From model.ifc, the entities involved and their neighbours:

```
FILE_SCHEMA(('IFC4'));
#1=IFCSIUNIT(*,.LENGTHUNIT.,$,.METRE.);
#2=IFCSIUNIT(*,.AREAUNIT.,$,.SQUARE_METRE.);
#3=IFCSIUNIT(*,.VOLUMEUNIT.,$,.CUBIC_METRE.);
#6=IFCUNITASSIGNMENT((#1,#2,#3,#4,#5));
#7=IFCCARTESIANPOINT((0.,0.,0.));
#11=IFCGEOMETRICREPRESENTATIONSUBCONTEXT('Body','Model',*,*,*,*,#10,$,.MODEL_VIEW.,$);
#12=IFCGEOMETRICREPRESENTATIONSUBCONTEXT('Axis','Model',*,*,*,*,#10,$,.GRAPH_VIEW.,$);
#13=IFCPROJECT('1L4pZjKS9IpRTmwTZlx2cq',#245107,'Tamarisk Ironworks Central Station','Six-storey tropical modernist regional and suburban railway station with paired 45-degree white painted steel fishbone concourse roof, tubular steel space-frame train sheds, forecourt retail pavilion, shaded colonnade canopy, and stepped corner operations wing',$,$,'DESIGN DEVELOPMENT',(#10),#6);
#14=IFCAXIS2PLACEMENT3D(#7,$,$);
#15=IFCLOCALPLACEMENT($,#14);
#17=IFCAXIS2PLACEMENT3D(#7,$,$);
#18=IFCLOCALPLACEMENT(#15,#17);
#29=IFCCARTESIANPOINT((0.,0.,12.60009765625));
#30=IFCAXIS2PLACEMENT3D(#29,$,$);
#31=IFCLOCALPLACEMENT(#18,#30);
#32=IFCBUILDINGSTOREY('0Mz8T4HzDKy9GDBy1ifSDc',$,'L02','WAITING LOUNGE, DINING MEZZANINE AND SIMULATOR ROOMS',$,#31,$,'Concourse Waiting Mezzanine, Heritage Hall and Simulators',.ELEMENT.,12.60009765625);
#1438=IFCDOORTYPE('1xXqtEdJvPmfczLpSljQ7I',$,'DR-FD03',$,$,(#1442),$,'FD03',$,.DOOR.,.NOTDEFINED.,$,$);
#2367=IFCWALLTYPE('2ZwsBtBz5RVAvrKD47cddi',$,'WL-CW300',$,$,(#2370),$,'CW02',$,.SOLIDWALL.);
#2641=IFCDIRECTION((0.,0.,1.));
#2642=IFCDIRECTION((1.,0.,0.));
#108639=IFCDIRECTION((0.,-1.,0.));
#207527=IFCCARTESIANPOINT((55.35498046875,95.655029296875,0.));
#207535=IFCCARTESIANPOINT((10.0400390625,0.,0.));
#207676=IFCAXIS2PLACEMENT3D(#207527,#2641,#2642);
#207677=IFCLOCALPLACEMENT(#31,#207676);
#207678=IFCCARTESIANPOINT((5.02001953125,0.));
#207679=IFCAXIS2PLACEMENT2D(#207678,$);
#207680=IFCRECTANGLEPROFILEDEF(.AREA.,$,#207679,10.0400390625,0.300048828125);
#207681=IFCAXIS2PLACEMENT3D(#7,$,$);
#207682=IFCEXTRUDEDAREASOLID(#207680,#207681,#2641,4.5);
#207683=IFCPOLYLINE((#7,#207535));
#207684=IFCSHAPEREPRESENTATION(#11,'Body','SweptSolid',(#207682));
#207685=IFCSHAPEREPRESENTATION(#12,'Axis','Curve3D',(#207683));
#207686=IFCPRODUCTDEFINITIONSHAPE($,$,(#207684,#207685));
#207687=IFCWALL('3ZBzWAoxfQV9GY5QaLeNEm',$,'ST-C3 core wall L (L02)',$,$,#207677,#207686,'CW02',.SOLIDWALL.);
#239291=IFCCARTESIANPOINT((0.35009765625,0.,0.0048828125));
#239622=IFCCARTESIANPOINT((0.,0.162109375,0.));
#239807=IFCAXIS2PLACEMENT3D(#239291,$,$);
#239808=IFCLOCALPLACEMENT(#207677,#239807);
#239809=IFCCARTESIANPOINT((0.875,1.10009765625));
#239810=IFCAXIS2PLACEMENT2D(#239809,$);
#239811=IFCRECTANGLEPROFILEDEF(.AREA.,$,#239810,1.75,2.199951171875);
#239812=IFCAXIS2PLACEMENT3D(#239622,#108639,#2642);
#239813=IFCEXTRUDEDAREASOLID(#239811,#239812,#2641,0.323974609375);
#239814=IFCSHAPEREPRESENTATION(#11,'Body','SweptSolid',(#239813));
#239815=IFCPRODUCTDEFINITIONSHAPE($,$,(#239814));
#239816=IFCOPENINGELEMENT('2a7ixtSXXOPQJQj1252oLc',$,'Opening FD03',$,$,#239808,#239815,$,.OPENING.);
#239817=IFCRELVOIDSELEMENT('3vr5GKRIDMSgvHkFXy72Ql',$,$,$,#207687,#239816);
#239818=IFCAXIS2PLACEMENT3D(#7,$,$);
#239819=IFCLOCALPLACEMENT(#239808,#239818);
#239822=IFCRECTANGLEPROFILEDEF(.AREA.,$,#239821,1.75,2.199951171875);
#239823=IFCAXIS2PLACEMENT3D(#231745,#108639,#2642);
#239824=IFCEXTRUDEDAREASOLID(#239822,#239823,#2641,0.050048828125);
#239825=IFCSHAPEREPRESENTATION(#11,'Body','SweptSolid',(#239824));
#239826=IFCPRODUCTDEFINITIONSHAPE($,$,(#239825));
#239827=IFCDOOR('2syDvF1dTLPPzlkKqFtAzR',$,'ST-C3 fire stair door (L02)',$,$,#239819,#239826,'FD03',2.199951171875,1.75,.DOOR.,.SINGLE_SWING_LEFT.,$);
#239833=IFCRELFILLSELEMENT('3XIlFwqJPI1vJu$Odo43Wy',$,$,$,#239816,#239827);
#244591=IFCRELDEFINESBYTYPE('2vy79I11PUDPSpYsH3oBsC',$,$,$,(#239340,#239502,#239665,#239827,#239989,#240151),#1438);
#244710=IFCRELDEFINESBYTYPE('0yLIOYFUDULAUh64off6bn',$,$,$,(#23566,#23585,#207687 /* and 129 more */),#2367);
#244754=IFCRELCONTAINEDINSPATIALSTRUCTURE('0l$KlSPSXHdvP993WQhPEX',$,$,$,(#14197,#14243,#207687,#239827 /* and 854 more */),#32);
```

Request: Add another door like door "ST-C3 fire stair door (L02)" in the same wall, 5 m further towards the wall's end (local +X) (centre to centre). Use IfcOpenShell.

```python
import ifcopenshell
import ifcopenshell.api.feature
import ifcopenshell.api.geometry
import ifcopenshell.api.root
import ifcopenshell.geom
import ifcopenshell.util.element
import ifcopenshell.util.placement
import ifcopenshell.util.shape
import ifcopenshell.util.unit

model = ifcopenshell.open("model.ifc")
unit_scale = ifcopenshell.util.unit.calculate_unit_scale(model)
settings = ifcopenshell.geom.settings()


def volume(element):
    """Net volume in cubic metres, openings subtracted."""
    shape = ifcopenshell.geom.create_shape(settings, element)
    return ifcopenshell.util.shape.get_volume(shape.geometry)


door = model.by_guid("2syDvF1dTLPPzlkKqFtAzR")
opening = door.FillsVoids[0].RelatingOpeningElement
wall = opening.VoidsElements[0].RelatingBuildingElement
before = volume(wall)
shift = ifcopenshell.util.placement.get_local_placement(wall.ObjectPlacement)[:3, 0] * 5 / unit_scale

# copy_class copies the void relationship, type, container and properties, but no geometry.
new_opening = ifcopenshell.api.root.copy_class(model, product=opening)
new_opening.Representation = ifcopenshell.util.element.copy_deep(
    model, opening.Representation, exclude=["IfcGeometricRepresentationContext", "IfcRepresentationMap"]
)
new_door = ifcopenshell.api.root.copy_class(model, product=door)
new_door.Representation = ifcopenshell.util.element.copy_deep(
    model, door.Representation, exclude=["IfcGeometricRepresentationContext", "IfcRepresentationMap"]
)
new_door.Tag = None
ifcopenshell.api.feature.add_filling(model, opening=new_opening, element=new_door)

for old, new in ((opening, new_opening), (door, new_door)):
    matrix = ifcopenshell.util.placement.get_local_placement(old.ObjectPlacement)
    matrix[:3, 3] += shift
    ifcopenshell.api.geometry.edit_object_placement(model, product=new, matrix=matrix, is_si=False)

after = volume(wall)

print(f"wall volume {before:.3f} -> {after:.3f} m3")

model.write("model_rev.ifc")
```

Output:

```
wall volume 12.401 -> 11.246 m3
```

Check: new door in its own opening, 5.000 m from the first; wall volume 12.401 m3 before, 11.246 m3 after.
